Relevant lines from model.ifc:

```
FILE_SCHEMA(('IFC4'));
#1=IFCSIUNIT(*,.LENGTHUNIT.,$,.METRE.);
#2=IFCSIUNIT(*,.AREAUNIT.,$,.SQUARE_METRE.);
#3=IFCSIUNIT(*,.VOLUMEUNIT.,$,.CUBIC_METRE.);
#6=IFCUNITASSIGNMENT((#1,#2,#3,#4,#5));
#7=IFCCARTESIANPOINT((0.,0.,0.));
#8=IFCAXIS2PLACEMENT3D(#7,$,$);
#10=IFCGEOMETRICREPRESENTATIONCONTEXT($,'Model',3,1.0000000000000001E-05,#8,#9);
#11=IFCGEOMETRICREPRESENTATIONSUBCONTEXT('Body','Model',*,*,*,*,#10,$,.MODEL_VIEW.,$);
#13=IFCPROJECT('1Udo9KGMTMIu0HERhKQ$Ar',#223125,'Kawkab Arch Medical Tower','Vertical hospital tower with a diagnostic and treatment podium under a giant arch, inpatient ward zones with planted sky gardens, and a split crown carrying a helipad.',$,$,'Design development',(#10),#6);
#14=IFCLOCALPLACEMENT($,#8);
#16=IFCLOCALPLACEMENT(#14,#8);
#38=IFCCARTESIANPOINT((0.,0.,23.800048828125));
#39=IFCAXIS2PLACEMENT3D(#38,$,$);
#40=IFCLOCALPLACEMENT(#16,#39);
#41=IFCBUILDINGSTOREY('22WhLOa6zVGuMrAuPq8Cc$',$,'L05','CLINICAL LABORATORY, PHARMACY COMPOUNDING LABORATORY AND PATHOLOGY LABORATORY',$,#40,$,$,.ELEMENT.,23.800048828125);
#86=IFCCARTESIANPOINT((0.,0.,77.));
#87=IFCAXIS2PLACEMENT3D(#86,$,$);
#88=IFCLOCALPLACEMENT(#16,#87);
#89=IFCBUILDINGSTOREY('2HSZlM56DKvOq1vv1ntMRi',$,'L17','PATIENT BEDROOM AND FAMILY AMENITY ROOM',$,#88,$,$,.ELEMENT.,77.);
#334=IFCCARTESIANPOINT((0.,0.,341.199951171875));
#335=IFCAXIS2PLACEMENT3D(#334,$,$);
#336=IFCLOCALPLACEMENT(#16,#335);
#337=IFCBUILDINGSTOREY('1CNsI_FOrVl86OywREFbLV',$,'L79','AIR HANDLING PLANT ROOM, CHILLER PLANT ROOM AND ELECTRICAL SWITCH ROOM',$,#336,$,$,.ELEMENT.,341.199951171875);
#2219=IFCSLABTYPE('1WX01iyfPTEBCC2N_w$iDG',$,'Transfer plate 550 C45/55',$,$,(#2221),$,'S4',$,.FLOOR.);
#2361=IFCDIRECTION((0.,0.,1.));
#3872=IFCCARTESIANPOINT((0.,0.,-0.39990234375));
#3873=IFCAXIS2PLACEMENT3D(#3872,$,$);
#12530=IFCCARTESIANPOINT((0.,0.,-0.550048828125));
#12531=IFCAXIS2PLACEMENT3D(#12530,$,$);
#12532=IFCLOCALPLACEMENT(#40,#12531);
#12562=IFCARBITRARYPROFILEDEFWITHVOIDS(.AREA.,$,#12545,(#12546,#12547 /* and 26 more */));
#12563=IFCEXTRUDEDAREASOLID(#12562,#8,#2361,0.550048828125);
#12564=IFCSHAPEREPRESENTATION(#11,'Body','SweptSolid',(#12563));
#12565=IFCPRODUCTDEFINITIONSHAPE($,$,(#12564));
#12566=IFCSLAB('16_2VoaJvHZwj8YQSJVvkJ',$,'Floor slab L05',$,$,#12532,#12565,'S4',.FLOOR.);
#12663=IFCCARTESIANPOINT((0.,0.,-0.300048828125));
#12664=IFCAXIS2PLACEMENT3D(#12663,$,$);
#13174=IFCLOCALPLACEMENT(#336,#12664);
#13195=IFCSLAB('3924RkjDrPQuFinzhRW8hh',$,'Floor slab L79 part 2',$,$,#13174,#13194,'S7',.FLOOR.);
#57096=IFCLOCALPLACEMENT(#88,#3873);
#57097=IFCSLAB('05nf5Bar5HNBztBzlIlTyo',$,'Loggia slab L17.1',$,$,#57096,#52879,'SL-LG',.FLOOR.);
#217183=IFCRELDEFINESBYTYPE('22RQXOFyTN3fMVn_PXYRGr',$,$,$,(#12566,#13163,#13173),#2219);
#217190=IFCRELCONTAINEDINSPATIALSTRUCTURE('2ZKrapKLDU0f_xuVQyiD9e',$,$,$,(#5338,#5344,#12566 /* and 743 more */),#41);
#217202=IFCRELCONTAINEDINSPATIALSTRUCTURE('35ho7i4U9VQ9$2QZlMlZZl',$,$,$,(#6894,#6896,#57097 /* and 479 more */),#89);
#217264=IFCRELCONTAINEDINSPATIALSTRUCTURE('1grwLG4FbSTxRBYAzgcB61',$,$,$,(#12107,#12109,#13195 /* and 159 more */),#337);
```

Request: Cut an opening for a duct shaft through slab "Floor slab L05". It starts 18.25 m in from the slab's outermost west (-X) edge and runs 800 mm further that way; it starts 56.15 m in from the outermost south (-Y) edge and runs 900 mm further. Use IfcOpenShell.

```python
import numpy as np
import ifcopenshell
import ifcopenshell.api.feature
import ifcopenshell.api.geometry
import ifcopenshell.api.root
import ifcopenshell.geom
import ifcopenshell.util.placement
import ifcopenshell.util.representation
import ifcopenshell.util.shape
import ifcopenshell.util.unit

model = ifcopenshell.open("model.ifc")
unit_scale = ifcopenshell.util.unit.calculate_unit_scale(model)
settings = ifcopenshell.geom.settings()


def volume(element):
    """Net volume in cubic metres, openings subtracted."""
    shape = ifcopenshell.geom.create_shape(settings, element)
    return ifcopenshell.util.shape.get_volume(shape.geometry)


slab = model.by_guid("16_2VoaJvHZwj8YQSJVvkJ")
before = volume(slab)

# Extent in the slab's own axes, in metres. The edges named are its -X and -Y sides.
slab_shape = ifcopenshell.geom.create_shape(settings, slab)
vertices = ifcopenshell.util.shape.get_vertices(slab_shape.geometry)
x_min, y_min, bottom = vertices.min(axis=0)
top = vertices[:, 2].max()

opening = ifcopenshell.api.root.create_entity(model, ifc_class="IfcOpeningElement", name="Duct shaft opening", predefined_type="OPENING")
context = ifcopenshell.util.representation.get_context(model, "Model", "Body", "MODEL_VIEW")
width, depth = 0.8, 0.9
outline = [(0.0, 0.0), (width, 0.0), (width, depth), (0.0, depth), (0.0, 0.0)]
# Overshoot both faces by 50 mm so the cut is clean.
shape = ifcopenshell.api.geometry.add_slab_representation(
    model, context=context, depth=top - bottom + 0.1, polyline=outline
)
ifcopenshell.api.geometry.assign_representation(model, product=opening, representation=shape)

matrix = ifcopenshell.util.placement.get_local_placement(slab.ObjectPlacement)
matrix[:, 3] = matrix @ np.append(np.array([x_min + 18.25, y_min + 56.15, bottom - 0.05]) / unit_scale, 1.0)
ifcopenshell.api.geometry.edit_object_placement(model, product=opening, matrix=matrix, is_si=False)
ifcopenshell.api.feature.add_feature(model, feature=opening, element=slab)

after = volume(slab)

print(f"slab volume {before:.3f} -> {after:.3f} m3")

model.write("model_v2.ifc")
```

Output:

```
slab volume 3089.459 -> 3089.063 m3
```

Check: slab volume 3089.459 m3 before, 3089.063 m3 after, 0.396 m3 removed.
